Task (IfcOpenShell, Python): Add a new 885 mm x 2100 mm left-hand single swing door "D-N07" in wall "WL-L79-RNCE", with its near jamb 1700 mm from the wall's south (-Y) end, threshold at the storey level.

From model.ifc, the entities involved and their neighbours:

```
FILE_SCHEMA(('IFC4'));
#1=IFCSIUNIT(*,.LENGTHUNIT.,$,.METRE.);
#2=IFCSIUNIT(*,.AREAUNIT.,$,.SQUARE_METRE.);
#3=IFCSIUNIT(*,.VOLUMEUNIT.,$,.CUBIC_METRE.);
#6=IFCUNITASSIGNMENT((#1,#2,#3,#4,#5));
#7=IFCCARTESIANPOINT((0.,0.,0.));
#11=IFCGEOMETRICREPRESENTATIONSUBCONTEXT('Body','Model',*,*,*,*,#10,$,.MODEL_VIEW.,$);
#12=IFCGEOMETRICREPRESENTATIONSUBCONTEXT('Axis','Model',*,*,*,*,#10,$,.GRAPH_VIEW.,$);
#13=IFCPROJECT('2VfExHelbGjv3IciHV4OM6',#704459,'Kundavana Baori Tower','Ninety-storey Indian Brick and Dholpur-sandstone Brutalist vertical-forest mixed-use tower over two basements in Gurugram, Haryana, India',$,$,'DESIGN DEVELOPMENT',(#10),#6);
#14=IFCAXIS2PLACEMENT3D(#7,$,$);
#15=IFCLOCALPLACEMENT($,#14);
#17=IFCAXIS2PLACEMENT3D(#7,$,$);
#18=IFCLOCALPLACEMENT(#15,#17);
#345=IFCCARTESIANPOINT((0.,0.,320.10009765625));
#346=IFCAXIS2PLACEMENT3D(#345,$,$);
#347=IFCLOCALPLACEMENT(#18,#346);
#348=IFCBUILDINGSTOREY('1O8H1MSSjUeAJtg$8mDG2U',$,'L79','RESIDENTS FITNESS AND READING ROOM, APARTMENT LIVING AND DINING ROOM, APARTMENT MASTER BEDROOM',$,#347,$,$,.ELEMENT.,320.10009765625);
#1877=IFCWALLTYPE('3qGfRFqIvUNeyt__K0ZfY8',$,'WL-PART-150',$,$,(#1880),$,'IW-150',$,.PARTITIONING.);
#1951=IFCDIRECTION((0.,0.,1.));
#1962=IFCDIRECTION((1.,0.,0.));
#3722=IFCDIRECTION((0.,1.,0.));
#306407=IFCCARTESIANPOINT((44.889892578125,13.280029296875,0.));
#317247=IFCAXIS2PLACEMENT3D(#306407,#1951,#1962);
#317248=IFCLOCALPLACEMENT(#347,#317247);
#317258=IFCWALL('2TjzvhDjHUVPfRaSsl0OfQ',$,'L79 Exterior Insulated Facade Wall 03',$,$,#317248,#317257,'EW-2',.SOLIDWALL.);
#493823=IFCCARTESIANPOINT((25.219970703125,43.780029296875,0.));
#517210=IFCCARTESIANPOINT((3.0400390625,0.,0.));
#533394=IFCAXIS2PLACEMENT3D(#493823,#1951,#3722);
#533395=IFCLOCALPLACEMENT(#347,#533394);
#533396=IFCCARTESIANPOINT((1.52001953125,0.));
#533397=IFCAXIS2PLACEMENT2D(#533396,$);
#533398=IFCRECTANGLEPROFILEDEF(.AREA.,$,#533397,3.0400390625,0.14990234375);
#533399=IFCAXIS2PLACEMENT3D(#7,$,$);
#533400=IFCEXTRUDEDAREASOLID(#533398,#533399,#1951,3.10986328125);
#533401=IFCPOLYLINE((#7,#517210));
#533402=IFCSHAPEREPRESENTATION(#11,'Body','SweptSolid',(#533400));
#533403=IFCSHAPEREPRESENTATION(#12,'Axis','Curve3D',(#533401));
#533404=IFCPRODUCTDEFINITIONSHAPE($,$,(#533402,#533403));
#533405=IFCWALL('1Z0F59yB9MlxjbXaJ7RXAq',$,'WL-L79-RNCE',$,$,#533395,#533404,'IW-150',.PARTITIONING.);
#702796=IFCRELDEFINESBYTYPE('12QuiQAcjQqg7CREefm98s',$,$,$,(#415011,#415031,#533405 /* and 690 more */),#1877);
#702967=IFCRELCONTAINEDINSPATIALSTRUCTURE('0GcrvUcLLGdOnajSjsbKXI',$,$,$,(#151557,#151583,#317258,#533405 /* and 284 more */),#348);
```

```python
import numpy as np
import ifcopenshell
import ifcopenshell.api.feature
import ifcopenshell.api.geometry
import ifcopenshell.api.root
import ifcopenshell.api.spatial
import ifcopenshell.geom
import ifcopenshell.util.element
import ifcopenshell.util.placement
import ifcopenshell.util.representation
import ifcopenshell.util.shape
import ifcopenshell.util.unit

model = ifcopenshell.open("model.ifc")
unit_scale = ifcopenshell.util.unit.calculate_unit_scale(model)
settings = ifcopenshell.geom.settings()


def volume(element):
    """Net volume in cubic metres, openings subtracted."""
    shape = ifcopenshell.geom.create_shape(settings, element)
    return ifcopenshell.util.shape.get_volume(shape.geometry)


wall = model.by_id(533405)
storey = ifcopenshell.util.element.get_container(wall, ifc_class="IfcBuildingStorey")
context = ifcopenshell.util.representation.get_context(model, "Model", "Body", "MODEL_VIEW")
before = volume(wall)

width, height, from_end, sill = 0.885, 2.1, 1.7, 0.0  # metres

# The wall runs along its own X axis, and the end named is its -X end.
wall_shape = ifcopenshell.geom.create_shape(settings, wall)
x, y, z = ifcopenshell.util.shape.get_vertices(wall_shape.geometry).T
start = x.min() + from_end
face, thickness = float(y.min()), float(y.max() - y.min())
wall_matrix = ifcopenshell.util.placement.get_local_placement(wall.ObjectPlacement)
level = ifcopenshell.util.placement.get_local_placement(storey.ObjectPlacement)[2, 3]


def in_wall(x, y):
    """Placement at x, y metres in the wall's axes, at sill height."""
    matrix = wall_matrix.copy()
    matrix[:, 3] = wall_matrix @ np.array([x / unit_scale, y / unit_scale, 0.0, 1.0])
    matrix[2, 3] = level + sill / unit_scale
    return matrix


# Opening: a box that overshoots both wall faces by 50 mm.
opening = ifcopenshell.api.root.create_entity(model, ifc_class="IfcOpeningElement", predefined_type="OPENING")
box = ifcopenshell.api.geometry.add_wall_representation(
    model, context=context, length=width, height=height, thickness=thickness + 0.1
)
ifcopenshell.api.geometry.assign_representation(model, product=opening, representation=box)
ifcopenshell.api.geometry.edit_object_placement(model, product=opening, matrix=in_wall(start, face - 0.05), is_si=False)
ifcopenshell.api.feature.add_feature(model, feature=opening, element=wall)

door = ifcopenshell.api.root.create_entity(model, ifc_class="IfcDoor", name="D-N07", predefined_type="DOOR")
door.OverallWidth, door.OverallHeight = width / unit_scale, height / unit_scale
door.OperationType = "SINGLE_SWING_LEFT"
body = ifcopenshell.api.geometry.add_door_representation(
    model,
    context=context,
    overall_width=door.OverallWidth,
    overall_height=door.OverallHeight,
    operation_type="SINGLE_SWING_LEFT",
    lining_properties={"LiningDepth": thickness / unit_scale, "ThresholdDepth": thickness / unit_scale},
)
ifcopenshell.api.geometry.assign_representation(model, product=door, representation=body)
ifcopenshell.api.spatial.assign_container(model, products=[door], relating_structure=storey)
ifcopenshell.api.feature.add_filling(model, opening=opening, element=door)

# The lining spans the wall, so the door starts at the wall face.
ifcopenshell.api.geometry.edit_object_placement(model, product=door, matrix=in_wall(start, face), is_si=False)

after = volume(wall)

print(f"wall volume {before:.3f} -> {after:.3f} m3")

model.write("model_v2.ifc")
```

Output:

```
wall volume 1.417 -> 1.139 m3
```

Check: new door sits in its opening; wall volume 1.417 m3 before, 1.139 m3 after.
